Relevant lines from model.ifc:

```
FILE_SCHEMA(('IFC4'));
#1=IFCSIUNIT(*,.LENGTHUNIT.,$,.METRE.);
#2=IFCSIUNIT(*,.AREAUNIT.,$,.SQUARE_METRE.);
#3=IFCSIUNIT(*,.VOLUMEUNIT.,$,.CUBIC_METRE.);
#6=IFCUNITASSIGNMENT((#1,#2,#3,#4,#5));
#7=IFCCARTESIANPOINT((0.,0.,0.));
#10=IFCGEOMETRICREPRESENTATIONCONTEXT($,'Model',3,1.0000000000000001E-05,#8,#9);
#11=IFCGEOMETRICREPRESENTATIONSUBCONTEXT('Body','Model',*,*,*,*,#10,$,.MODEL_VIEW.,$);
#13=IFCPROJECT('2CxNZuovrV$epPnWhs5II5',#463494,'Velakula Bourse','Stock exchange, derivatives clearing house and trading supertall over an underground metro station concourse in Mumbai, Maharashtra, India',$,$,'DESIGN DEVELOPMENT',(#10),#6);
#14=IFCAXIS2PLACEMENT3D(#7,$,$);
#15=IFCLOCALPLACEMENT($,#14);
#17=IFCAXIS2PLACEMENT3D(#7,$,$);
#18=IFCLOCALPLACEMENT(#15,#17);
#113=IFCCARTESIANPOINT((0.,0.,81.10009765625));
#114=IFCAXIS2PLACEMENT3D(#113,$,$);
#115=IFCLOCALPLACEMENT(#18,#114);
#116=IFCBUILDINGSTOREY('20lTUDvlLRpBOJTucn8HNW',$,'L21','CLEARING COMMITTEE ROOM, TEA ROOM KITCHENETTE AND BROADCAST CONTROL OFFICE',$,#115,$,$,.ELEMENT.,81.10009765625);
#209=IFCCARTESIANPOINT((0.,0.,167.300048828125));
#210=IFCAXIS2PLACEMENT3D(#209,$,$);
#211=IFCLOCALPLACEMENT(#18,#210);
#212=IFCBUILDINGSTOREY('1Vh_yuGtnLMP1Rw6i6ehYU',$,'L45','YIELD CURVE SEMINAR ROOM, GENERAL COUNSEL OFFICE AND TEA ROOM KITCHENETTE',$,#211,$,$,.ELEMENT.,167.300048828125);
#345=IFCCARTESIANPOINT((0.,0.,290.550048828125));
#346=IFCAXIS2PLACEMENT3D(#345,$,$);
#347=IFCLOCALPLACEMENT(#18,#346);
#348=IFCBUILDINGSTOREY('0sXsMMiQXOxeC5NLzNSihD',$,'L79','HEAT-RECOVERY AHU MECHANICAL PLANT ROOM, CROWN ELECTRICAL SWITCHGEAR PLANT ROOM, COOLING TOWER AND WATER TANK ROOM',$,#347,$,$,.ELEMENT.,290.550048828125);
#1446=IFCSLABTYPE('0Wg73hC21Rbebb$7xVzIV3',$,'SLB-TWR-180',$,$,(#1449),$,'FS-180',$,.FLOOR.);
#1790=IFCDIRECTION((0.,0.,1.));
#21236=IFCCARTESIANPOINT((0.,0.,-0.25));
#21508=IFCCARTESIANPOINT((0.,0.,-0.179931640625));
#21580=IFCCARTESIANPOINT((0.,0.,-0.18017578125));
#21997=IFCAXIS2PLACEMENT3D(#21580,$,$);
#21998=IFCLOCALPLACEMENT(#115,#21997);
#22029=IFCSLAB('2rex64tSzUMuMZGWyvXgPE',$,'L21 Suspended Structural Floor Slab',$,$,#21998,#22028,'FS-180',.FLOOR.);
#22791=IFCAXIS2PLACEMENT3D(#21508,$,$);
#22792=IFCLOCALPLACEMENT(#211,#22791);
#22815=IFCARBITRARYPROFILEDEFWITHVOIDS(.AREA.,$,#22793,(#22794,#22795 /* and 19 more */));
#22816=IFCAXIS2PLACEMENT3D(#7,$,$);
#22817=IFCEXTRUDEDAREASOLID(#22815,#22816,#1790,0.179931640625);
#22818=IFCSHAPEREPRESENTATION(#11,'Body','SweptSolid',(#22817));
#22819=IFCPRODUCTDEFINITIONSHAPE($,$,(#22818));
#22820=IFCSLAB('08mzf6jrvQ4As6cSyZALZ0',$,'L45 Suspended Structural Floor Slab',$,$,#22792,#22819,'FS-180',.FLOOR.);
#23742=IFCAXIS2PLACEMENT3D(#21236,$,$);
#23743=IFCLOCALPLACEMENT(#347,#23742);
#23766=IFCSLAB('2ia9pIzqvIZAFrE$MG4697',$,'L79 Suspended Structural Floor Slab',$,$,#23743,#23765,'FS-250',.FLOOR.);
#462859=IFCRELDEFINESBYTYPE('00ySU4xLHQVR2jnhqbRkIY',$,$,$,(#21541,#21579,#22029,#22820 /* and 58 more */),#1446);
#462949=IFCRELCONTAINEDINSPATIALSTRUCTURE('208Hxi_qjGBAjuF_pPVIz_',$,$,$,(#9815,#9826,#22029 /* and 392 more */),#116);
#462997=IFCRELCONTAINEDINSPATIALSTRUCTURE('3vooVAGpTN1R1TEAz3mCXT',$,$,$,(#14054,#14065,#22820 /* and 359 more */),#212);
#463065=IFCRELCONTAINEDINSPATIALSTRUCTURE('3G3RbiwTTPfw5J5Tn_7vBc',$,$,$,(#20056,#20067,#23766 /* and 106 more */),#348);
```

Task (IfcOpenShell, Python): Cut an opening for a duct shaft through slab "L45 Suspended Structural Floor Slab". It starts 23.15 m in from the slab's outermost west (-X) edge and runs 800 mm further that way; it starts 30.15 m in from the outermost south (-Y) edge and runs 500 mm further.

```python
import numpy as np
import ifcopenshell
import ifcopenshell.api.feature
import ifcopenshell.api.geometry
import ifcopenshell.api.root
import ifcopenshell.geom
import ifcopenshell.util.placement
import ifcopenshell.util.representation
import ifcopenshell.util.shape
import ifcopenshell.util.unit

model = ifcopenshell.open("model.ifc")
unit_scale = ifcopenshell.util.unit.calculate_unit_scale(model)
settings = ifcopenshell.geom.settings()


def volume(element):
    """Net volume in cubic metres, openings subtracted."""
    shape = ifcopenshell.geom.create_shape(settings, element)
    return ifcopenshell.util.shape.get_volume(shape.geometry)


slab = model.by_id(22820)
before = volume(slab)

# Extent in the slab's own axes, in metres. The edges named are its -X and -Y sides.
slab_shape = ifcopenshell.geom.create_shape(settings, slab)
vertices = ifcopenshell.util.shape.get_vertices(slab_shape.geometry)
x_min, y_min, bottom = vertices.min(axis=0)
top = vertices[:, 2].max()

opening = ifcopenshell.api.root.create_entity(model, ifc_class="IfcOpeningElement", name="Duct shaft opening", predefined_type="OPENING")
context = ifcopenshell.util.representation.get_context(model, "Model", "Body", "MODEL_VIEW")
width, depth = 0.8, 0.5
outline = [(0.0, 0.0), (width, 0.0), (width, depth), (0.0, depth), (0.0, 0.0)]
# Overshoot both faces by 50 mm so the cut is clean.
shape = ifcopenshell.api.geometry.add_slab_representation(
    model, context=context, depth=top - bottom + 0.1, polyline=outline
)
ifcopenshell.api.geometry.assign_representation(model, product=opening, representation=shape)

matrix = ifcopenshell.util.placement.get_local_placement(slab.ObjectPlacement)
matrix[:, 3] = matrix @ np.append(np.array([x_min + 23.15, y_min + 30.15, bottom - 0.05]) / unit_scale, 1.0)
ifcopenshell.api.geometry.edit_object_placement(model, product=opening, matrix=matrix, is_si=False)
ifcopenshell.api.feature.add_feature(model, feature=opening, element=slab)

after = volume(slab)

print(f"slab volume {before:.3f} -> {after:.3f} m3")

model.write("model_edited.ifc")
```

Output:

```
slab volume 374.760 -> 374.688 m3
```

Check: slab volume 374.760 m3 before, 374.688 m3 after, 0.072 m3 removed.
